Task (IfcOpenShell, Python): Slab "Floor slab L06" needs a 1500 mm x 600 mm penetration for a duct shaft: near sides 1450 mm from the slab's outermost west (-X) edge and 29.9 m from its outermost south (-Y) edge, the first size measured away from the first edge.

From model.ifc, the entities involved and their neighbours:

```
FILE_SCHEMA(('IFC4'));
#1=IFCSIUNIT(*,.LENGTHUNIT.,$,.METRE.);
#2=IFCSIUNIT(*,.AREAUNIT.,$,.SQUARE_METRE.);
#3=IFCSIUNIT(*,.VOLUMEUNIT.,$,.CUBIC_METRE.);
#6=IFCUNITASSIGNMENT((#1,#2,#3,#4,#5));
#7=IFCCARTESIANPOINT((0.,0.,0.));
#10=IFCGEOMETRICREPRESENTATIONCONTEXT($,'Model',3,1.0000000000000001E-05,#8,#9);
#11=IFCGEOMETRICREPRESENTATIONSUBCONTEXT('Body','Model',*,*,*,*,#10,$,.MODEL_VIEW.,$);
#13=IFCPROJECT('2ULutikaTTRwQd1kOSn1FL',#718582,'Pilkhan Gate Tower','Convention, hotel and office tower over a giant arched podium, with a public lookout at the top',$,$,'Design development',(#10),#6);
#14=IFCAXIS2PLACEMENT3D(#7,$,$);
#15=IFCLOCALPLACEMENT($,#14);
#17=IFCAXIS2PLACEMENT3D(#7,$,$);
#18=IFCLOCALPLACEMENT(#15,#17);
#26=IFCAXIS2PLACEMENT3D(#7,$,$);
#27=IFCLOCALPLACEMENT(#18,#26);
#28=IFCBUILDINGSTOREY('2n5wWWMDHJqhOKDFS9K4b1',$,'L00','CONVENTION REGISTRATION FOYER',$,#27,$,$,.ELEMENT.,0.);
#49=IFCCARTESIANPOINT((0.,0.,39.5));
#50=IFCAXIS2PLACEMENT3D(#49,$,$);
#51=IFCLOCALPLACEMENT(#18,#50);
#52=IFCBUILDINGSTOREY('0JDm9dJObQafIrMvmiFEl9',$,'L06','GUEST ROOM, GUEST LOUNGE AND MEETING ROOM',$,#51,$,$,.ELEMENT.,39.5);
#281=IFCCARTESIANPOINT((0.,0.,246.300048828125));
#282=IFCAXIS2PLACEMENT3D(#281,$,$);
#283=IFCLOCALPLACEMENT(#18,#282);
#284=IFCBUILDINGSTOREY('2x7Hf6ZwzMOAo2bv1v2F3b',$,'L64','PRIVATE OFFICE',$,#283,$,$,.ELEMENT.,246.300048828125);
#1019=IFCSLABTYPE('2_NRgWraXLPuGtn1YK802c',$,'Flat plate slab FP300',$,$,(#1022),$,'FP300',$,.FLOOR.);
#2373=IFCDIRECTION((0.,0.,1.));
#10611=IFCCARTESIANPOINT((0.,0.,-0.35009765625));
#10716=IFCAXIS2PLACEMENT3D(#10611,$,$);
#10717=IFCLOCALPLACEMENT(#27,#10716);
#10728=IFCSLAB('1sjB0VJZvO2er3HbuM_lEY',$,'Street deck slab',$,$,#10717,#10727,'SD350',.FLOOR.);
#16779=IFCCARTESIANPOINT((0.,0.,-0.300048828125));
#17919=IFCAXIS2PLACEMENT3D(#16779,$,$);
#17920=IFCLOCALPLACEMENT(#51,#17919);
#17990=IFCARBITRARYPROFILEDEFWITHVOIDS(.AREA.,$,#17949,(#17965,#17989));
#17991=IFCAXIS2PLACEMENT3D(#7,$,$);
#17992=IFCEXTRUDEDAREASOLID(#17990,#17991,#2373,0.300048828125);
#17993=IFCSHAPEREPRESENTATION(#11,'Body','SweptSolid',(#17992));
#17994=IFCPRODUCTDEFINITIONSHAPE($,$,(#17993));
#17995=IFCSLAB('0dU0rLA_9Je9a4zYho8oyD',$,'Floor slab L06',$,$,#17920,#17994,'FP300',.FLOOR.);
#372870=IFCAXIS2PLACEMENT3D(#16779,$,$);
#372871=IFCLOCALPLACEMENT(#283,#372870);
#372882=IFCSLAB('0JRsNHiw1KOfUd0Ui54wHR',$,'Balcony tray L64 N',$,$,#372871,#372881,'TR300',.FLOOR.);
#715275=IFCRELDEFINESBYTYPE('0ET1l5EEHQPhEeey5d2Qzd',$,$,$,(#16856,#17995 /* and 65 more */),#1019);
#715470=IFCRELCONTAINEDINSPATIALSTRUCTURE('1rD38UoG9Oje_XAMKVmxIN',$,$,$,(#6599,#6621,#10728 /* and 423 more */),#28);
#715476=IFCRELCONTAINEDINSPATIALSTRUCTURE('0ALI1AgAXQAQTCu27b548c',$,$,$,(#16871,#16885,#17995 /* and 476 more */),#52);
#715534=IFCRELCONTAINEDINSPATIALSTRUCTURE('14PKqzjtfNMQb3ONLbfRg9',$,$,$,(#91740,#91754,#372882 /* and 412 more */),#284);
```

```python
import numpy as np
import ifcopenshell
import ifcopenshell.api.feature
import ifcopenshell.api.geometry
import ifcopenshell.api.root
import ifcopenshell.geom
import ifcopenshell.util.placement
import ifcopenshell.util.representation
import ifcopenshell.util.shape
import ifcopenshell.util.unit

model = ifcopenshell.open("model.ifc")
unit_scale = ifcopenshell.util.unit.calculate_unit_scale(model)
settings = ifcopenshell.geom.settings()


def volume(element):
    """Net volume in cubic metres, openings subtracted."""
    shape = ifcopenshell.geom.create_shape(settings, element)
    return ifcopenshell.util.shape.get_volume(shape.geometry)


slab = model.by_id(17995)
before = volume(slab)

# Extent in the slab's own axes, in metres. The edges named are its -X and -Y sides.
slab_shape = ifcopenshell.geom.create_shape(settings, slab)
vertices = ifcopenshell.util.shape.get_vertices(slab_shape.geometry)
x_min, y_min, bottom = vertices.min(axis=0)
top = vertices[:, 2].max()

opening = ifcopenshell.api.root.create_entity(model, ifc_class="IfcOpeningElement", name="Duct shaft opening", predefined_type="OPENING")
context = ifcopenshell.util.representation.get_context(model, "Model", "Body", "MODEL_VIEW")
width, depth = 1.5, 0.6
outline = [(0.0, 0.0), (width, 0.0), (width, depth), (0.0, depth), (0.0, 0.0)]
# Overshoot both faces by 50 mm so the cut is clean.
shape = ifcopenshell.api.geometry.add_slab_representation(
    model, context=context, depth=top - bottom + 0.1, polyline=outline
)
ifcopenshell.api.geometry.assign_representation(model, product=opening, representation=shape)

matrix = ifcopenshell.util.placement.get_local_placement(slab.ObjectPlacement)
matrix[:, 3] = matrix @ np.append(np.array([x_min + 1.45, y_min + 29.9, bottom - 0.05]) / unit_scale, 1.0)
ifcopenshell.api.geometry.edit_object_placement(model, product=opening, matrix=matrix, is_si=False)
ifcopenshell.api.feature.add_feature(model, feature=opening, element=slab)

after = volume(slab)

print(f"slab volume {before:.3f} -> {after:.3f} m3")

model.write("model_rev.ifc")
```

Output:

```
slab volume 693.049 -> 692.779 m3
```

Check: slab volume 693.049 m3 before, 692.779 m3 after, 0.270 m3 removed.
